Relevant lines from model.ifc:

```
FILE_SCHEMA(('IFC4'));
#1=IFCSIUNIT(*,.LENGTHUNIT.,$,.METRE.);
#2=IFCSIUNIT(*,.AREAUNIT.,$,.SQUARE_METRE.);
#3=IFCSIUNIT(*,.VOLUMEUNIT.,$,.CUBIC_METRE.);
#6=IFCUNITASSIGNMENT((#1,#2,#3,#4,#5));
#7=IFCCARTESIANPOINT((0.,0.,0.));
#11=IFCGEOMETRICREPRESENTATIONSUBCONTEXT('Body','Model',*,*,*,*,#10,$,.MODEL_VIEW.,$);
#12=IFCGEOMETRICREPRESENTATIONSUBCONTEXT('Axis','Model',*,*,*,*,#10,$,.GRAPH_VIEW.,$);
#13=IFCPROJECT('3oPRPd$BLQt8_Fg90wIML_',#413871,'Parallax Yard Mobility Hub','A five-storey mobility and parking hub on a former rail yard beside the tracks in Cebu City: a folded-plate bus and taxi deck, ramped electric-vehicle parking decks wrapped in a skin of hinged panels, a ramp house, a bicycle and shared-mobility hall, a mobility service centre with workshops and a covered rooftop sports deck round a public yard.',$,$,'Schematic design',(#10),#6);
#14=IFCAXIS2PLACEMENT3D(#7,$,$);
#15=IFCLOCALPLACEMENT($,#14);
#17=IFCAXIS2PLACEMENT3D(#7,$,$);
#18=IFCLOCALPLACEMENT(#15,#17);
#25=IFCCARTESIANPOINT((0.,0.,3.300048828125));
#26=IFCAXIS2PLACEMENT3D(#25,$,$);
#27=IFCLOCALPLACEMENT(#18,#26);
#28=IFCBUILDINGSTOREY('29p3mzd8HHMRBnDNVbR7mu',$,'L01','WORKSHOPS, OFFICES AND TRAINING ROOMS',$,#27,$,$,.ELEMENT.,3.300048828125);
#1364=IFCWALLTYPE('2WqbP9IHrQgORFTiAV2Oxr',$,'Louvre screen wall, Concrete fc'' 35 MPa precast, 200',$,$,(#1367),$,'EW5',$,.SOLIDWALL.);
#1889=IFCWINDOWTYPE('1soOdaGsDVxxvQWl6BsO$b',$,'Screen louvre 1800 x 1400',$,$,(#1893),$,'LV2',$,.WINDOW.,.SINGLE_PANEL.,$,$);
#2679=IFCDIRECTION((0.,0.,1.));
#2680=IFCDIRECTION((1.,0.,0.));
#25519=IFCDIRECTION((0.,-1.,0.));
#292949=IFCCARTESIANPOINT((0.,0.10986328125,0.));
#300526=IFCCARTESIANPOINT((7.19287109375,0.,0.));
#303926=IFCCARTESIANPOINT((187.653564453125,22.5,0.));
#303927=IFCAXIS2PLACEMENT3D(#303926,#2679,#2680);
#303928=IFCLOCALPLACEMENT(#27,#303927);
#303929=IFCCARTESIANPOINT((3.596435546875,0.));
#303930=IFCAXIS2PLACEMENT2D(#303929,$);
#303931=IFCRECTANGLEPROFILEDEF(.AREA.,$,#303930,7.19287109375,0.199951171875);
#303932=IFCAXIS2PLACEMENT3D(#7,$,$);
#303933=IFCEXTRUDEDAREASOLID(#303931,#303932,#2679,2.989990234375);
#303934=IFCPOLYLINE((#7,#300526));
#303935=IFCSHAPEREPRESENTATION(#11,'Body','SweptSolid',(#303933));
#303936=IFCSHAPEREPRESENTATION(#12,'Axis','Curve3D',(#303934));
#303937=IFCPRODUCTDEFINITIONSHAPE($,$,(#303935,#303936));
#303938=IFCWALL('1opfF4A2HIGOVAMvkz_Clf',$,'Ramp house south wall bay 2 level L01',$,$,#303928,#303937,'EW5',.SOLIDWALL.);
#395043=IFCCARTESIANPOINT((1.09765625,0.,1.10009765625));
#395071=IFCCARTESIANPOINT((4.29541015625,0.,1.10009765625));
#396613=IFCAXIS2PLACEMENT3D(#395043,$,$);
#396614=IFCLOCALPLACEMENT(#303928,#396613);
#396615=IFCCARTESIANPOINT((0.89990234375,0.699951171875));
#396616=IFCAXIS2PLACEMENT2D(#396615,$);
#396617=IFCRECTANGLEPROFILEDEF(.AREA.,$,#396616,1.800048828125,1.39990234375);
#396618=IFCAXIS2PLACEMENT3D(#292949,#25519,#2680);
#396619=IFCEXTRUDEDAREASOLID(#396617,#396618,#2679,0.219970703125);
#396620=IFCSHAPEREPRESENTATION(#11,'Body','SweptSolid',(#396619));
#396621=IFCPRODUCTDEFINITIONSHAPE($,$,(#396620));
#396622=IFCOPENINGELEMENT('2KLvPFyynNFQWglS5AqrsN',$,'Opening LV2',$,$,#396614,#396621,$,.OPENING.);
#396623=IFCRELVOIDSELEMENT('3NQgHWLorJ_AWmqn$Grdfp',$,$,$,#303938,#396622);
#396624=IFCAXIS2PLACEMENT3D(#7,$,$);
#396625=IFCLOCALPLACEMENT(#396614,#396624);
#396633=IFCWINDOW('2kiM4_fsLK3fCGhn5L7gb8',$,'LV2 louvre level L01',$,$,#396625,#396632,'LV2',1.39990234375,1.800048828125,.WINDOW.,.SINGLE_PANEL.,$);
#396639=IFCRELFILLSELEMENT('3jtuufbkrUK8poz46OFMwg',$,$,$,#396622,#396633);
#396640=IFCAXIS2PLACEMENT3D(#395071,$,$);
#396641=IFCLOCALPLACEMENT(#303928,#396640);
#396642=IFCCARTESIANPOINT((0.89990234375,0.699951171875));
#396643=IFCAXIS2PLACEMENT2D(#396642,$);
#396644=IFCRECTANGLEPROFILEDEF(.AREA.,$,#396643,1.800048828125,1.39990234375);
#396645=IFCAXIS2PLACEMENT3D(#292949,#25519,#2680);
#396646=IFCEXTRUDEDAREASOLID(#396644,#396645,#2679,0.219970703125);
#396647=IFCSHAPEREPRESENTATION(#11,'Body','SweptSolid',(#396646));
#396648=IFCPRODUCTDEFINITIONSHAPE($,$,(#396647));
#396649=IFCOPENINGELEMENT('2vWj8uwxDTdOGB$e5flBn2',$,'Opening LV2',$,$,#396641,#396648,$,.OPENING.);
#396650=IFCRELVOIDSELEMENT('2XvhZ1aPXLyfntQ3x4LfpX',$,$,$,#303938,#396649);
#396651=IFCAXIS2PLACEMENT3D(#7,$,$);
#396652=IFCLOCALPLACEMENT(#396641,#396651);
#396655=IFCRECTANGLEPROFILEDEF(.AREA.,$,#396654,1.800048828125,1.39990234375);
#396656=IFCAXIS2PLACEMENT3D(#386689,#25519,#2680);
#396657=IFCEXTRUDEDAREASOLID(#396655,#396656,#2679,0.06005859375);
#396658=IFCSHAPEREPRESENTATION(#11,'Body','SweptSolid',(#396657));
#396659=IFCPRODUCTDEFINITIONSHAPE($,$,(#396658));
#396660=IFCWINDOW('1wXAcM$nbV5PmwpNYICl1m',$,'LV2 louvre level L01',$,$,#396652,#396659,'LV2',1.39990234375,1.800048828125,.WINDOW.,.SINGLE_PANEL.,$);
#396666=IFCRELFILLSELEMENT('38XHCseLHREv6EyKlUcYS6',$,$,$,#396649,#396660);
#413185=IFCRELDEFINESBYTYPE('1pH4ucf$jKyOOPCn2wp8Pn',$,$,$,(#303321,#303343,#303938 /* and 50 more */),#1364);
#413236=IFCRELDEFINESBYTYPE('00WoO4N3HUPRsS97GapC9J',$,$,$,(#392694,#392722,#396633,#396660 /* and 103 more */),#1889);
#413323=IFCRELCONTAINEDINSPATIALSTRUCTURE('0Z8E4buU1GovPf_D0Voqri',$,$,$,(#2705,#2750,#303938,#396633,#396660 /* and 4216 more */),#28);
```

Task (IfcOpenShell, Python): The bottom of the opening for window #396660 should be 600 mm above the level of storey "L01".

```python
import numpy as np
import ifcopenshell
import ifcopenshell.api.geometry
import ifcopenshell.geom
import ifcopenshell.util.element
import ifcopenshell.util.placement
import ifcopenshell.util.shape
import ifcopenshell.util.unit

model = ifcopenshell.open("model.ifc")
unit_scale = ifcopenshell.util.unit.calculate_unit_scale(model)

window = model.by_guid("1wXAcM$nbV5PmwpNYICl1m")
opening = window.FillsVoids[0].RelatingOpeningElement
storey = ifcopenshell.util.element.get_container(window, ifc_class="IfcBuildingStorey")
level = ifcopenshell.util.placement.get_local_placement(storey.ObjectPlacement)[2, 3]

# The opening's origin need not be at the sill, so measure its lowest point.
shape = ifcopenshell.geom.create_shape(ifcopenshell.geom.settings(), opening)
bottom = ifcopenshell.util.shape.get_shape_bottom_elevation(shape, shape.geometry) / unit_scale
dz = level + 0.6 - bottom

shift = np.array([0.0, 0.0, dz])
# The window is placed relative to its opening, so it follows when the opening moves.
matrix = ifcopenshell.util.placement.get_local_placement(opening.ObjectPlacement)
matrix[:3, 3] += shift
ifcopenshell.api.geometry.edit_object_placement(
    model, product=opening, matrix=matrix, is_si=False, should_transform_children=True
)

print(f"moved by {dz * unit_scale:+.3f} m")

model.write("model_updated.ifc")
```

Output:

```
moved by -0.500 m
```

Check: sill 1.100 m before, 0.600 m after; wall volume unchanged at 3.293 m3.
